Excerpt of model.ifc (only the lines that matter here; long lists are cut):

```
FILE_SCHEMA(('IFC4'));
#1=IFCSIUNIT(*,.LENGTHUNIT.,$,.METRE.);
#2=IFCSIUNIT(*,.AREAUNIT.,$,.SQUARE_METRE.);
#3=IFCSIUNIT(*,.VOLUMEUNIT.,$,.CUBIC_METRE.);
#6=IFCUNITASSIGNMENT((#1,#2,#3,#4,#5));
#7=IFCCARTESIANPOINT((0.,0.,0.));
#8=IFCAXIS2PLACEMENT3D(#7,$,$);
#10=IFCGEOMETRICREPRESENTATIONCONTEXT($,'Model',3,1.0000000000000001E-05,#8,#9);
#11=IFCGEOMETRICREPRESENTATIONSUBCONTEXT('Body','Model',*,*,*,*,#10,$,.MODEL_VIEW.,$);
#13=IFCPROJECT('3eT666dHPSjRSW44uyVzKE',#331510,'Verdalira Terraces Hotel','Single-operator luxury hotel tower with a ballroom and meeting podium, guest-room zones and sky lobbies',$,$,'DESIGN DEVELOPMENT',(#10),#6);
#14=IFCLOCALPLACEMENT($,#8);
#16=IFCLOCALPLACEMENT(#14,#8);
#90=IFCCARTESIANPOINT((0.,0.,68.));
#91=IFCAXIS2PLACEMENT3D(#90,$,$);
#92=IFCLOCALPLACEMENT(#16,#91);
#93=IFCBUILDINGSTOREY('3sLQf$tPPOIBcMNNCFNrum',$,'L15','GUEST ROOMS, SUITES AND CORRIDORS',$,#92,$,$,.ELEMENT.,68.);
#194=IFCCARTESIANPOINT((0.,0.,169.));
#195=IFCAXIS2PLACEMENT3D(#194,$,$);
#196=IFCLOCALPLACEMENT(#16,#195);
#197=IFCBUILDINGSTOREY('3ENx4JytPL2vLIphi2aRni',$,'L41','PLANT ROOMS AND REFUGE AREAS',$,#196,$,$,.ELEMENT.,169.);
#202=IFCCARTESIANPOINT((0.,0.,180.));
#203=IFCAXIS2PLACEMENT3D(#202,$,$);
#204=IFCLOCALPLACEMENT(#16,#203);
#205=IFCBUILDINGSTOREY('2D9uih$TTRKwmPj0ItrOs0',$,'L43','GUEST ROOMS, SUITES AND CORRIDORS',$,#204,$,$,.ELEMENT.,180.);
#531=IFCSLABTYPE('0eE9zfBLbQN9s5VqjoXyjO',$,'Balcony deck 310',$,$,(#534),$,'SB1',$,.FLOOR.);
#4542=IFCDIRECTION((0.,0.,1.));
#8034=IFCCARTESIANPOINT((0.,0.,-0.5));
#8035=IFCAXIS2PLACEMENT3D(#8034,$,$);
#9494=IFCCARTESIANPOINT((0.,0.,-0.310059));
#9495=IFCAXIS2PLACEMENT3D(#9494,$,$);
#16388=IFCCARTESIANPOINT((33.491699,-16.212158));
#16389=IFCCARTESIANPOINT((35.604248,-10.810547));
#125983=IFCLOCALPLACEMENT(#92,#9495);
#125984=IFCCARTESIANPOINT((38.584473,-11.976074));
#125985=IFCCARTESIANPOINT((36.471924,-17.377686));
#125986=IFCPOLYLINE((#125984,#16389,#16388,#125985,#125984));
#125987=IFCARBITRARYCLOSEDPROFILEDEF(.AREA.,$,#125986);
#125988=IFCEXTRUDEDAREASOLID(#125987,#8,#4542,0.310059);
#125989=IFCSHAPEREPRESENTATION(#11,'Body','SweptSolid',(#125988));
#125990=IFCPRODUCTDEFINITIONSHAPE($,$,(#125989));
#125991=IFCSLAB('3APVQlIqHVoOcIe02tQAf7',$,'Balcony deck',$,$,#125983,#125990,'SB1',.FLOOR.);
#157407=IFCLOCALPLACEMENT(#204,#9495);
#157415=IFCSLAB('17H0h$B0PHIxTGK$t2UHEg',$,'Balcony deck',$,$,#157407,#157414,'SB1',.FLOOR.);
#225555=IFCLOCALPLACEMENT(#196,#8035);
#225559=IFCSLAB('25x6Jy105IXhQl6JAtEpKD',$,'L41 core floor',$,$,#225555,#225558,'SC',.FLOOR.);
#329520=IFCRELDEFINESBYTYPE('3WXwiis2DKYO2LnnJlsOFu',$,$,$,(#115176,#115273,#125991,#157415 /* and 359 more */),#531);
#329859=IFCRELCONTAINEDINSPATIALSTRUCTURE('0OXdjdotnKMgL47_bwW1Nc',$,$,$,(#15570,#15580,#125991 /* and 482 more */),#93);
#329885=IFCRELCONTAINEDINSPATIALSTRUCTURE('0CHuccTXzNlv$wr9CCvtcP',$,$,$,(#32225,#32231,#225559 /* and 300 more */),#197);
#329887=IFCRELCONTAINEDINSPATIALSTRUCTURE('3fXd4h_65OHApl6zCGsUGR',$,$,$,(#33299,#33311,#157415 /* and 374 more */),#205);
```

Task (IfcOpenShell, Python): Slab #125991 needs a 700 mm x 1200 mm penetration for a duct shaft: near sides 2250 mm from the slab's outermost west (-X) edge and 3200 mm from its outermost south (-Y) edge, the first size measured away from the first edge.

```python
import numpy as np
import ifcopenshell
import ifcopenshell.api.feature
import ifcopenshell.api.geometry
import ifcopenshell.api.root
import ifcopenshell.geom
import ifcopenshell.util.placement
import ifcopenshell.util.representation
import ifcopenshell.util.shape
import ifcopenshell.util.unit

model = ifcopenshell.open("model.ifc")
unit_scale = ifcopenshell.util.unit.calculate_unit_scale(model)
settings = ifcopenshell.geom.settings()


def volume(element):
    """Net volume in cubic metres, openings subtracted."""
    shape = ifcopenshell.geom.create_shape(settings, element)
    return ifcopenshell.util.shape.get_volume(shape.geometry)


slab = model.by_guid("3APVQlIqHVoOcIe02tQAf7")
before = volume(slab)

# Extent in the slab's own axes, in metres. The edges named are its -X and -Y sides.
slab_shape = ifcopenshell.geom.create_shape(settings, slab)
vertices = ifcopenshell.util.shape.get_vertices(slab_shape.geometry)
x_min, y_min, bottom = vertices.min(axis=0)
top = vertices[:, 2].max()

opening = ifcopenshell.api.root.create_entity(model, ifc_class="IfcOpeningElement", name="Duct shaft opening", predefined_type="OPENING")
context = ifcopenshell.util.representation.get_context(model, "Model", "Body", "MODEL_VIEW")
width, depth = 0.7, 1.2
outline = [(0.0, 0.0), (width, 0.0), (width, depth), (0.0, depth), (0.0, 0.0)]
# Overshoot both faces by 50 mm so the cut is clean.
shape = ifcopenshell.api.geometry.add_slab_representation(
    model, context=context, depth=top - bottom + 0.1, polyline=outline
)
ifcopenshell.api.geometry.assign_representation(model, product=opening, representation=shape)

matrix = ifcopenshell.util.placement.get_local_placement(slab.ObjectPlacement)
matrix[:, 3] = matrix @ np.append(np.array([x_min + 2.25, y_min + 3.2, bottom - 0.05]) / unit_scale, 1.0)
ifcopenshell.api.geometry.edit_object_placement(model, product=opening, matrix=matrix, is_si=False)
ifcopenshell.api.feature.add_feature(model, feature=opening, element=slab)

after = volume(slab)

print(f"slab volume {before:.3f} -> {after:.3f} m3")

model.write("model_updated.ifc")
```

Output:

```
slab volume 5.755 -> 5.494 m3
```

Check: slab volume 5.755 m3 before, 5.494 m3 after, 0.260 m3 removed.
